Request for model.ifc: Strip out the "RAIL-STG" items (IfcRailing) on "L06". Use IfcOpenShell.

First a look at what the model holds.

```python
import ifcopenshell
import ifcopenshell.util.element

model = ifcopenshell.open("model.ifc")
print(model.schema)
storey = next(s for s in model.by_type("IfcBuildingStorey") if s.Name == "L06")
railings = [e for e in ifcopenshell.util.element.get_decomposition(storey) if e.is_a("IfcRailing")]
seen = {}
for e in railings:
    element_type = ifcopenshell.util.element.get_type(e)
    name = element_type.Name if element_type not in (None, e) else None
    seen[name] = seen.get(name, 0) + 1
for name, count in sorted(seen.items(), key=str):
    print(count, "x", name)
```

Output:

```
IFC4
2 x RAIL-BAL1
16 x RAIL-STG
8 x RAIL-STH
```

```python
import ifcopenshell
import ifcopenshell.api.root
import ifcopenshell.util.element

model = ifcopenshell.open("model.ifc")

storey = next(s for s in model.by_type("IfcBuildingStorey") if s.Name == "L06")
railings = [e for e in ifcopenshell.util.element.get_decomposition(storey) if e.is_a("IfcRailing")]
targets = [e for e in railings if (t := ifcopenshell.util.element.get_type(e)) not in (None, e) and t.Name == "RAIL-STG"]

for e in targets:
    ifcopenshell.api.root.remove_product(model, product=e)
print(len(targets), "removed")

model.write("model_rev.ifc")
```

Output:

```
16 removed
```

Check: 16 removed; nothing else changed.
